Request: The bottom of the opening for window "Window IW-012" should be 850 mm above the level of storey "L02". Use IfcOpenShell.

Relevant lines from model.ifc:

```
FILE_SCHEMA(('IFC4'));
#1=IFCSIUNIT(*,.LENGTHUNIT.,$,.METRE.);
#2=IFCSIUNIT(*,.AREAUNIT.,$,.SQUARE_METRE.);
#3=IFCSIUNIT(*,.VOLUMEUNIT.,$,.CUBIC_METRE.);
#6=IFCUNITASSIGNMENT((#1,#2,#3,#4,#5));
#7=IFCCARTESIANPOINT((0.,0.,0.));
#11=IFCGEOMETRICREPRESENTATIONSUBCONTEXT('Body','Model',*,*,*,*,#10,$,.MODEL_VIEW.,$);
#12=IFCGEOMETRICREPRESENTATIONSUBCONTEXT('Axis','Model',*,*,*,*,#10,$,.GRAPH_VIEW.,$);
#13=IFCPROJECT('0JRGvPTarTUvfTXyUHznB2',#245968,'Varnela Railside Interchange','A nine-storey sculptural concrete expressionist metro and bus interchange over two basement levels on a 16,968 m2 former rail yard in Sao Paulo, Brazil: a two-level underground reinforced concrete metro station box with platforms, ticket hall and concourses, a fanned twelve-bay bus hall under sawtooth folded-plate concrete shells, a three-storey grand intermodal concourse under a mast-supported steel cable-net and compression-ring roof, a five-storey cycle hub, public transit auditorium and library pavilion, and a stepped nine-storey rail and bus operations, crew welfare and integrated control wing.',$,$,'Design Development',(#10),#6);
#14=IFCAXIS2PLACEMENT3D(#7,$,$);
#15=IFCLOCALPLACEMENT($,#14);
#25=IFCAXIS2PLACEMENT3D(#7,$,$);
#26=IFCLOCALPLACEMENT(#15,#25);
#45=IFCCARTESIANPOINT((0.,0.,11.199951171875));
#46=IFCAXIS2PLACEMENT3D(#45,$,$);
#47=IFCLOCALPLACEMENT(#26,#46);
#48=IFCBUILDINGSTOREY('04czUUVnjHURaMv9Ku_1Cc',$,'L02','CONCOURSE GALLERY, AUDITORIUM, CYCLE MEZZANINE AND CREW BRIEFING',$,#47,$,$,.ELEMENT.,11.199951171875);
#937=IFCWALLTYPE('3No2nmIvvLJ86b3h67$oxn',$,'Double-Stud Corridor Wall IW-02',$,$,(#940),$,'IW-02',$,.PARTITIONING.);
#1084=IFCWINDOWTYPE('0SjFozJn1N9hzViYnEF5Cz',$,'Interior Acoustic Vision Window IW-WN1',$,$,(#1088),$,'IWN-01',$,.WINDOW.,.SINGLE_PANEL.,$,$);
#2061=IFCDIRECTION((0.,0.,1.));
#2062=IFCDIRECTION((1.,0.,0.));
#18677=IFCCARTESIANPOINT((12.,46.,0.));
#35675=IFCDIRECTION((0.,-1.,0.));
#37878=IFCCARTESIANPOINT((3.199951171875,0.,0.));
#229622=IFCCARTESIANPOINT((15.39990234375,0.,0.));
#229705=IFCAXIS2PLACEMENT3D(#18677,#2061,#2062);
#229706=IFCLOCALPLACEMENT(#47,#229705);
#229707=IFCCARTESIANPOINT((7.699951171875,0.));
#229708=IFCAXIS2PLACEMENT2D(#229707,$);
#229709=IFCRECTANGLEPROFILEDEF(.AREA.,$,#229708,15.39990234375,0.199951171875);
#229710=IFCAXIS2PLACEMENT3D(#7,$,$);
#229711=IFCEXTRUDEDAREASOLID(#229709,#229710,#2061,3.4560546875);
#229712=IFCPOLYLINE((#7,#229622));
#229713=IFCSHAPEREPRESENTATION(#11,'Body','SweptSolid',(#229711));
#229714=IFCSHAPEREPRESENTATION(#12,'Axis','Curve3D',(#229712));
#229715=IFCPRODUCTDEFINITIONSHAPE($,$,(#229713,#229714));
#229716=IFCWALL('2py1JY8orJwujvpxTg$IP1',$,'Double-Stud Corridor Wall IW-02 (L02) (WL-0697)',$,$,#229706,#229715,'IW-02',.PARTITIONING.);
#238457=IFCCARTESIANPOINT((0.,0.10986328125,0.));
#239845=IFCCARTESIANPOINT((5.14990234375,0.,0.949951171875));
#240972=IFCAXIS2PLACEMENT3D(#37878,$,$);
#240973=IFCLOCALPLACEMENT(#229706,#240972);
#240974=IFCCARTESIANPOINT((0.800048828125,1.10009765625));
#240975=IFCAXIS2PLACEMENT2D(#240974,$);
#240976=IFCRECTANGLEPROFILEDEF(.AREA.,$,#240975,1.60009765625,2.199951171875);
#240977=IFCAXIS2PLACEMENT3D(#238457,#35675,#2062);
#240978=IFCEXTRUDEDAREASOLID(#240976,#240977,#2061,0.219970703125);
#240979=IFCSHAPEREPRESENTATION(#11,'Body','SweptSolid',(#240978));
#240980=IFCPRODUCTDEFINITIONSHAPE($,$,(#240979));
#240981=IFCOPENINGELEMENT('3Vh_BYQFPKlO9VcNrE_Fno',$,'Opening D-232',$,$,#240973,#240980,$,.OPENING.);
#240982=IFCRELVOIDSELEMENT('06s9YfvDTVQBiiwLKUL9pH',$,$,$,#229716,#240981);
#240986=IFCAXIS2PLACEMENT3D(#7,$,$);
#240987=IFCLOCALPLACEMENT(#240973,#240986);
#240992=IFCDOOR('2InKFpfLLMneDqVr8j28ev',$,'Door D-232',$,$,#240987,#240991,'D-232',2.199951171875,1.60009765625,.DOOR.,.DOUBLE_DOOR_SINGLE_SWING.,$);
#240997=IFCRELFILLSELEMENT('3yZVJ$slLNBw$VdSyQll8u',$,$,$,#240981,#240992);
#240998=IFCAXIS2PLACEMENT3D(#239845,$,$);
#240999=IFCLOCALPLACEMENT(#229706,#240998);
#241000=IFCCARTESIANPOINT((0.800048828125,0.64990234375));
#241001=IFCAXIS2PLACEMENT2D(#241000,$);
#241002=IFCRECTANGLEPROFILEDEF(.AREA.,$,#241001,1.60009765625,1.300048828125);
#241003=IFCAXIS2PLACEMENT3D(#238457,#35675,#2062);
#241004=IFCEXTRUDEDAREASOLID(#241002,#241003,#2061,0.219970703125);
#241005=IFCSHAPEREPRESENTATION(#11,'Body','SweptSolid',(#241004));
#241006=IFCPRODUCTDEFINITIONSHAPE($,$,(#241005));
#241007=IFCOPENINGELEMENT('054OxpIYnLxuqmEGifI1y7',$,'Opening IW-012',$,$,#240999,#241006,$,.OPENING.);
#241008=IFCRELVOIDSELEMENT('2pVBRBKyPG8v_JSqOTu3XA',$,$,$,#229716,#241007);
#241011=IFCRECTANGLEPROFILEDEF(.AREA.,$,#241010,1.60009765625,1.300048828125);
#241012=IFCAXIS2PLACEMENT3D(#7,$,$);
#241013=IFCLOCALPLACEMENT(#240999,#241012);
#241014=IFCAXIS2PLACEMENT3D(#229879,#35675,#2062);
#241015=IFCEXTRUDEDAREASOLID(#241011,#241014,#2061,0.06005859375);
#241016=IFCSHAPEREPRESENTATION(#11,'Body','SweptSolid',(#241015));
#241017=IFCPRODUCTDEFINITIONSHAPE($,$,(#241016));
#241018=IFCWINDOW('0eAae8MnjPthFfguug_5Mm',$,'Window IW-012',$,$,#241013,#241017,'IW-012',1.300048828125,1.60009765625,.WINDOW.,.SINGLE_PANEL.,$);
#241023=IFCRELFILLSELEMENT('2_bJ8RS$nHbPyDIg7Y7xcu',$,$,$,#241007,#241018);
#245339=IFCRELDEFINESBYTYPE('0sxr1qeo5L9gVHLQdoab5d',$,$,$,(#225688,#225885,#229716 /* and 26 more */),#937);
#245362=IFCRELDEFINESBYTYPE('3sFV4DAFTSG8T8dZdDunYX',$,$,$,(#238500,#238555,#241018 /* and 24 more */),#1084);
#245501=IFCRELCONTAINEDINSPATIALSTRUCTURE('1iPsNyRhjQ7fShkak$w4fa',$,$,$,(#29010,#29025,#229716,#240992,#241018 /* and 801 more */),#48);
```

```python
import numpy as np
import ifcopenshell
import ifcopenshell.api.geometry
import ifcopenshell.geom
import ifcopenshell.util.element
import ifcopenshell.util.placement
import ifcopenshell.util.shape
import ifcopenshell.util.unit

model = ifcopenshell.open("model.ifc")
unit_scale = ifcopenshell.util.unit.calculate_unit_scale(model)

window = model.by_guid("0eAae8MnjPthFfguug_5Mm")
opening = window.FillsVoids[0].RelatingOpeningElement
storey = ifcopenshell.util.element.get_container(window, ifc_class="IfcBuildingStorey")
level = ifcopenshell.util.placement.get_local_placement(storey.ObjectPlacement)[2, 3]

# The opening's origin need not be at the sill, so measure its lowest point.
shape = ifcopenshell.geom.create_shape(ifcopenshell.geom.settings(), opening)
bottom = ifcopenshell.util.shape.get_shape_bottom_elevation(shape, shape.geometry) / unit_scale
dz = level + 0.85 / unit_scale - bottom

shift = np.array([0.0, 0.0, dz])
# The window is placed relative to its opening, so it follows when the opening moves.
matrix = ifcopenshell.util.placement.get_local_placement(opening.ObjectPlacement)
matrix[:3, 3] += shift
ifcopenshell.api.geometry.edit_object_placement(
    model, product=opening, matrix=matrix, is_si=False, should_transform_children=True
)

print(f"moved by {dz * unit_scale:+.3f} m")

model.write("model_rev.ifc")
```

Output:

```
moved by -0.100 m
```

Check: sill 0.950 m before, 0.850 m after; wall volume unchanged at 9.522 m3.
